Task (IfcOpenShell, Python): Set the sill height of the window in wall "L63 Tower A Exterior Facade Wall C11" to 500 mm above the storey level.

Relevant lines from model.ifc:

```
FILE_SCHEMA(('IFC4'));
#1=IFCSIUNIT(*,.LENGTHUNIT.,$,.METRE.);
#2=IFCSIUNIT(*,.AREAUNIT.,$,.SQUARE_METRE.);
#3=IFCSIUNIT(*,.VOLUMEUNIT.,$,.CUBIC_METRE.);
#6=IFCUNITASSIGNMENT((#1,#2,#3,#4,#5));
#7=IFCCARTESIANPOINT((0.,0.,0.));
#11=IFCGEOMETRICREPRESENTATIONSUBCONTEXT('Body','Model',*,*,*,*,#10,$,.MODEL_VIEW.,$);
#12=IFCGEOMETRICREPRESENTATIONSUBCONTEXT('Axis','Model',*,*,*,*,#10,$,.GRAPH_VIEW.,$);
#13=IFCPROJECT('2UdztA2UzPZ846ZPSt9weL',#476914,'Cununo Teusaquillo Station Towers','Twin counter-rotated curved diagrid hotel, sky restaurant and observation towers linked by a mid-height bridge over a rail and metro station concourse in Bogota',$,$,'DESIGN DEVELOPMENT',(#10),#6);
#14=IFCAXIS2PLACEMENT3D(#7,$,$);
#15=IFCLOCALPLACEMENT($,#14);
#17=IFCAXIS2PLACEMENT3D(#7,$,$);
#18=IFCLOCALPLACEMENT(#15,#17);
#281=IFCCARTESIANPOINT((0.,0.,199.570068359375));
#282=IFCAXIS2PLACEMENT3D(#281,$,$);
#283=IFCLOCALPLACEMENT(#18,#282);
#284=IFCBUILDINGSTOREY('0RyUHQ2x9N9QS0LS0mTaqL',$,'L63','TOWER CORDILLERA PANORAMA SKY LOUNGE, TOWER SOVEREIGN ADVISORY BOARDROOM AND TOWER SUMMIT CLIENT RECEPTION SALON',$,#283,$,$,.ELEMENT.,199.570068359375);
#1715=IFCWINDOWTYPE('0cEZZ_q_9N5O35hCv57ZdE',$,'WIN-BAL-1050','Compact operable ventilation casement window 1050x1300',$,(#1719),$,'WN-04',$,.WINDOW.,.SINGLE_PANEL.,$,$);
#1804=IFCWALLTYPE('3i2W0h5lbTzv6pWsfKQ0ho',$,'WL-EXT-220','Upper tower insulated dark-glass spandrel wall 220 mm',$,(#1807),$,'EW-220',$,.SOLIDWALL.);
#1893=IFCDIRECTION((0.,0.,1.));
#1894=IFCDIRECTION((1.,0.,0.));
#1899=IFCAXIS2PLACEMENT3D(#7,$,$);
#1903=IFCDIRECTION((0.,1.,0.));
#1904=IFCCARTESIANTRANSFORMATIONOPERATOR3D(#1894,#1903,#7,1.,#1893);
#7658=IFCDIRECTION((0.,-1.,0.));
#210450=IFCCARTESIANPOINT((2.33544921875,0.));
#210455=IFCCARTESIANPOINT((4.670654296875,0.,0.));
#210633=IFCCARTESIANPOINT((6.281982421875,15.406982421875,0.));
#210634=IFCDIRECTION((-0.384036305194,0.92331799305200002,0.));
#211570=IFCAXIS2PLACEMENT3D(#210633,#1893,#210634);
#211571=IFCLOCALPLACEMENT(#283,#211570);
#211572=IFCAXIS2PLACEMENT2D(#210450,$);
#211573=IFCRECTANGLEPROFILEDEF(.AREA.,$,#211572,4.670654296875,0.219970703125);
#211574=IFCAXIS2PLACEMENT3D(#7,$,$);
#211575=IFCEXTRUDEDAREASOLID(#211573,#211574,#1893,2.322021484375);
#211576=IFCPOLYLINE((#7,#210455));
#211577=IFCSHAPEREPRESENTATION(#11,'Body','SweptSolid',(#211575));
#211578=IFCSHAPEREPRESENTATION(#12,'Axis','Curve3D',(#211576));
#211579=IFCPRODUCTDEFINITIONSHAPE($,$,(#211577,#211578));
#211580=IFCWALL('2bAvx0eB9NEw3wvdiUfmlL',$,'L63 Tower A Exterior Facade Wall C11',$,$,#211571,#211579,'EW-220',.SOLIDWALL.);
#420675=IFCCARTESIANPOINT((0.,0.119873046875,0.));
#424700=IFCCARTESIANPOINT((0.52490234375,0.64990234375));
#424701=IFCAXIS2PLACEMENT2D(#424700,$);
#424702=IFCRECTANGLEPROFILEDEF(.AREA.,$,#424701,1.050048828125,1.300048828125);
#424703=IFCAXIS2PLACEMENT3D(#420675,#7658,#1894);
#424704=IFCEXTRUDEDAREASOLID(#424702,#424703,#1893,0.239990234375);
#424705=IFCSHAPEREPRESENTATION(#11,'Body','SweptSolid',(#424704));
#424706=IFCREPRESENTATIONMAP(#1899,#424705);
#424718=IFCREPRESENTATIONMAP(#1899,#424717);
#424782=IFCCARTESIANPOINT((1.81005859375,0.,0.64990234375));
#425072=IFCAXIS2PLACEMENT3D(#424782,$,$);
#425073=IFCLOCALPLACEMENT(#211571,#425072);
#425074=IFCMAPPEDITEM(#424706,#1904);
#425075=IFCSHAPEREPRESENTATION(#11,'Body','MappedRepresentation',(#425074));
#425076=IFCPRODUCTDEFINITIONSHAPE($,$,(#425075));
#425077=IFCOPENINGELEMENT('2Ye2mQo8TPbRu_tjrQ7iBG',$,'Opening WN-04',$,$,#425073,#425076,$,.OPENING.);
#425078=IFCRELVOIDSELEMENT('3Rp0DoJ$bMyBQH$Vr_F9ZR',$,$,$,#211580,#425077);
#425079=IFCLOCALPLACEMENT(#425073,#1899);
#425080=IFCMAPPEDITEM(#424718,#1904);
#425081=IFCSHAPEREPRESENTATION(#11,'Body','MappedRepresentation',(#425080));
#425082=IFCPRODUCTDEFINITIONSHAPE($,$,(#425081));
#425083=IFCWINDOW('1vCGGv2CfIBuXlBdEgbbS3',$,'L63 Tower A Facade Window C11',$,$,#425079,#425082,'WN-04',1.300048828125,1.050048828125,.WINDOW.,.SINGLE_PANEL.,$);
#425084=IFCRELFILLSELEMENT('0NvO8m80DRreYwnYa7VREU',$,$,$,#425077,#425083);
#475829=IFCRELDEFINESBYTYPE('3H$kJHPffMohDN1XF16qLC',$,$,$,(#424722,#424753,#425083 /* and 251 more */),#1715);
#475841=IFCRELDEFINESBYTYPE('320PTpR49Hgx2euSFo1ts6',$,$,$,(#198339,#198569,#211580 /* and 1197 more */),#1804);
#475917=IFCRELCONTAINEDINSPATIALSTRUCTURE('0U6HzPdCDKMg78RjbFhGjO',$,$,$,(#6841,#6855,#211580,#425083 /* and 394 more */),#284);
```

```python
import numpy as np
import ifcopenshell
import ifcopenshell.api.geometry
import ifcopenshell.geom
import ifcopenshell.util.element
import ifcopenshell.util.placement
import ifcopenshell.util.shape
import ifcopenshell.util.unit

model = ifcopenshell.open("model.ifc")
unit_scale = ifcopenshell.util.unit.calculate_unit_scale(model)

window = model.by_guid("1vCGGv2CfIBuXlBdEgbbS3")
opening = window.FillsVoids[0].RelatingOpeningElement
storey = ifcopenshell.util.element.get_container(window, ifc_class="IfcBuildingStorey")
level = ifcopenshell.util.placement.get_local_placement(storey.ObjectPlacement)[2, 3]

# The opening's origin need not be at the sill, so measure its lowest point.
shape = ifcopenshell.geom.create_shape(ifcopenshell.geom.settings(), opening)
bottom = ifcopenshell.util.shape.get_shape_bottom_elevation(shape, shape.geometry) / unit_scale
dz = level + 0.5 - bottom

shift = np.array([0.0, 0.0, dz])
# The window is placed relative to its opening, so it follows when the opening moves.
matrix = ifcopenshell.util.placement.get_local_placement(opening.ObjectPlacement)
matrix[:3, 3] += shift
ifcopenshell.api.geometry.edit_object_placement(
    model, product=opening, matrix=matrix, is_si=False, should_transform_children=True
)

print(f"moved by {dz * unit_scale:+.3f} m")

model.write("model_v2.ifc")
```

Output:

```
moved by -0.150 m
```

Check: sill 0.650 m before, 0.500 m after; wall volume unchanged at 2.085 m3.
